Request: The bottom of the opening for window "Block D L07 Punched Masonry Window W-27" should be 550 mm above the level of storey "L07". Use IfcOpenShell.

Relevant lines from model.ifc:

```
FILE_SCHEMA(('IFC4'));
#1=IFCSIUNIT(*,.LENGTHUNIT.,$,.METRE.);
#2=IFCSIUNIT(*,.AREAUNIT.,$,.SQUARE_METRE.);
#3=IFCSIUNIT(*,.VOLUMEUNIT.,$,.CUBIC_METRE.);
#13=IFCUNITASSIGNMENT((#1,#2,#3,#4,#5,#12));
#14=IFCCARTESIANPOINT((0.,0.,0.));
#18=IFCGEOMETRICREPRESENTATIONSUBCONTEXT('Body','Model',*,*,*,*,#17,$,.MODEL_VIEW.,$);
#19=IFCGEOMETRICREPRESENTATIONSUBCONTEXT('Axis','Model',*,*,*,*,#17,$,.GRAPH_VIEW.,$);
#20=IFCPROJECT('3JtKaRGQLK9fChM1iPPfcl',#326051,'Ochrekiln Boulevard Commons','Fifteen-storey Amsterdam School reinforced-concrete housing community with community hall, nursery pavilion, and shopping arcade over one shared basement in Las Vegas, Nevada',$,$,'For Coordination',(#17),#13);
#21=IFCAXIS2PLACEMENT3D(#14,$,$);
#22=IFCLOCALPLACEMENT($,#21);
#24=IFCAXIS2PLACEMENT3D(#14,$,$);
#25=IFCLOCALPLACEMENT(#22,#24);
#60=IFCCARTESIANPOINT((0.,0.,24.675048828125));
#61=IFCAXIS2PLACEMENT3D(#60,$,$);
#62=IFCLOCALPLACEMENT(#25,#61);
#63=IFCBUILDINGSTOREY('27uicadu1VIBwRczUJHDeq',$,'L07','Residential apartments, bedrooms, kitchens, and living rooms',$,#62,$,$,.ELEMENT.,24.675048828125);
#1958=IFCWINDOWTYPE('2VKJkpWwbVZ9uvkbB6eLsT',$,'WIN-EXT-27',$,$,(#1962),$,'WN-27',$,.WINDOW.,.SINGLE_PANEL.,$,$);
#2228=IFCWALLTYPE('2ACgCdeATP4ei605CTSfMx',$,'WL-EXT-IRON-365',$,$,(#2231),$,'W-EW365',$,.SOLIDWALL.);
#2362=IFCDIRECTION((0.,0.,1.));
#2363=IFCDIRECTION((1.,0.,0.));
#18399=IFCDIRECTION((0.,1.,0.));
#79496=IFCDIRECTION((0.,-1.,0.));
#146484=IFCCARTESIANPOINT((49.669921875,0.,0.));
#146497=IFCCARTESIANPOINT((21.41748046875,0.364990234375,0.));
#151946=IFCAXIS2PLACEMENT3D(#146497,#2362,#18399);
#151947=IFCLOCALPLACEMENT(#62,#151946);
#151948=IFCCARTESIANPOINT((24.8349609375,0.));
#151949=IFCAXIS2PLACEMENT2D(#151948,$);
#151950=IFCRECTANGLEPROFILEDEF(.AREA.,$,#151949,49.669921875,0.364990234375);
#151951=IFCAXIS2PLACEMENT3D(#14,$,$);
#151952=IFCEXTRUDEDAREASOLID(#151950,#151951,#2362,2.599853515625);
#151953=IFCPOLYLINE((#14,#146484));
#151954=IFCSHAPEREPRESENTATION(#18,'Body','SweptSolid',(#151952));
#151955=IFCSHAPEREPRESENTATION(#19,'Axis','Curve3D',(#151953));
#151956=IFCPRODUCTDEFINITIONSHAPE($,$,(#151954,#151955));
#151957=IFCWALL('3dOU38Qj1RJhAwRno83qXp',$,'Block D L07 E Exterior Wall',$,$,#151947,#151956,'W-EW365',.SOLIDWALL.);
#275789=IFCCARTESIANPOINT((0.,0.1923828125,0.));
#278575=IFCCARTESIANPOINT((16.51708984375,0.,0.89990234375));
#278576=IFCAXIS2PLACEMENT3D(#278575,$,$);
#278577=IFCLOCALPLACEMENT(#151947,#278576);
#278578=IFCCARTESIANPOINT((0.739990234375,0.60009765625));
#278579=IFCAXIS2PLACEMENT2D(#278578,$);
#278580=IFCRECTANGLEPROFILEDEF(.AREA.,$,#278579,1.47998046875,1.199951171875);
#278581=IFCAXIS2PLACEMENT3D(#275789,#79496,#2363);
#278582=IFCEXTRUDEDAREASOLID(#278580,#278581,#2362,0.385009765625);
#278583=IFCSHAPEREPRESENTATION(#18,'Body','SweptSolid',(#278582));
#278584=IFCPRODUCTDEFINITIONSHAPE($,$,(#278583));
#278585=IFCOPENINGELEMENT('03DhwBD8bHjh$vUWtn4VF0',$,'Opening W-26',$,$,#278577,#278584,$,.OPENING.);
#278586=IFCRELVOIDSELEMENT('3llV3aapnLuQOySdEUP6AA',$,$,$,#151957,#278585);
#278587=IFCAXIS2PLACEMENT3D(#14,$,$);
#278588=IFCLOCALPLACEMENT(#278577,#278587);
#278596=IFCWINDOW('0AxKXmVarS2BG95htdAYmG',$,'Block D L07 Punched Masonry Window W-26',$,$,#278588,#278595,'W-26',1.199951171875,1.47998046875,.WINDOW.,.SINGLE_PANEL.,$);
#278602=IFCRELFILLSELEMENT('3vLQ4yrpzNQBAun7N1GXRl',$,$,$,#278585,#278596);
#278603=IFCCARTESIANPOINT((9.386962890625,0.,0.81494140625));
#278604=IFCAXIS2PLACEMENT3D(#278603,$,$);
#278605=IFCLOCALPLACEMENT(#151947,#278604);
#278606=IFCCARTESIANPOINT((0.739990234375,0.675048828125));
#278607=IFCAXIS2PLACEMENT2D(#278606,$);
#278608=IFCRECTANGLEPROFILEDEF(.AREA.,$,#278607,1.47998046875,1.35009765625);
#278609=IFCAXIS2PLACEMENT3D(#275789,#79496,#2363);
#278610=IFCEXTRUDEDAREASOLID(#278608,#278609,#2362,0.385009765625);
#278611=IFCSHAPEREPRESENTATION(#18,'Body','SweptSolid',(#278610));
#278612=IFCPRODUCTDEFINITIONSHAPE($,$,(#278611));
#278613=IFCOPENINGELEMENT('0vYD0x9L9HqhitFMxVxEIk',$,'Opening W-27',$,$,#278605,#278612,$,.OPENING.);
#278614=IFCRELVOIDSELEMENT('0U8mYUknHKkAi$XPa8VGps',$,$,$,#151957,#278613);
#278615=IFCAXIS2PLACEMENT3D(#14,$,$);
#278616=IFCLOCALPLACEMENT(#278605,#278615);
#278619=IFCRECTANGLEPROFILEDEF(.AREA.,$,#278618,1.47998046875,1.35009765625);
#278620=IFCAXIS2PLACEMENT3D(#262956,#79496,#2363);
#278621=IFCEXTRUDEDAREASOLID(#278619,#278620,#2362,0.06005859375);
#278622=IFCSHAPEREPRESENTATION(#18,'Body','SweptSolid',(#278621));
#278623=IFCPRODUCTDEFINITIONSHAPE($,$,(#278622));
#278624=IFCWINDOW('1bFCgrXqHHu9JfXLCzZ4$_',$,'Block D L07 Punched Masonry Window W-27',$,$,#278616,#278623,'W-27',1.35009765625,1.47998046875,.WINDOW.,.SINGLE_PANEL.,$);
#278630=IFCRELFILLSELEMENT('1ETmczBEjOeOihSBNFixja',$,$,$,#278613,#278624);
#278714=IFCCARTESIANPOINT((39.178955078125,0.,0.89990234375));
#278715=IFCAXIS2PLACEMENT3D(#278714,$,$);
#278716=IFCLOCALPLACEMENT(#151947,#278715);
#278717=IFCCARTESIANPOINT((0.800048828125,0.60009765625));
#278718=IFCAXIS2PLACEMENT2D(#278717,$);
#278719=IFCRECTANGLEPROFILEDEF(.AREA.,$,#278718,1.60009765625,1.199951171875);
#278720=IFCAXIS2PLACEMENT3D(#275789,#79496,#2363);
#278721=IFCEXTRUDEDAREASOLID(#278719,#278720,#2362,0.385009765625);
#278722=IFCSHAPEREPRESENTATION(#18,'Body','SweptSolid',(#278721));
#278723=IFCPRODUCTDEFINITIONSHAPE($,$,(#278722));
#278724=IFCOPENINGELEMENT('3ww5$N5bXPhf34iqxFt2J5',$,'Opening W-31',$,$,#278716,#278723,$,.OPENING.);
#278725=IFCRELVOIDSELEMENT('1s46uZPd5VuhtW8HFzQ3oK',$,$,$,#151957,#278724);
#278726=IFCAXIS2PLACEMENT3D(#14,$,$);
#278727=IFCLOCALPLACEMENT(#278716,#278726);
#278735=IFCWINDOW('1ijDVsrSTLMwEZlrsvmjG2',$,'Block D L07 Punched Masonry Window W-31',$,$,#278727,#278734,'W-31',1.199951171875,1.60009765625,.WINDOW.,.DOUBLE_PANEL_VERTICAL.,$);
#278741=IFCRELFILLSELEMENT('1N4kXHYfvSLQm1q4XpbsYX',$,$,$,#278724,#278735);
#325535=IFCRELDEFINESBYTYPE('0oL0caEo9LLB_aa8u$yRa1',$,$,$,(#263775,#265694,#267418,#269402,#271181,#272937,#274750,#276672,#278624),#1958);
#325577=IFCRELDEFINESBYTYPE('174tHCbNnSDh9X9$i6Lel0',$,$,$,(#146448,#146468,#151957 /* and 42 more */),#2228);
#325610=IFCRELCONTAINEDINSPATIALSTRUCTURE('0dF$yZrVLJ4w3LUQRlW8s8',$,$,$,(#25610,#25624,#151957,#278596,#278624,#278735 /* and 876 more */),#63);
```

```python
import numpy as np
import ifcopenshell
import ifcopenshell.api.geometry
import ifcopenshell.geom
import ifcopenshell.util.element
import ifcopenshell.util.placement
import ifcopenshell.util.shape
import ifcopenshell.util.unit

model = ifcopenshell.open("model.ifc")
unit_scale = ifcopenshell.util.unit.calculate_unit_scale(model)

window = model.by_id(278624)
opening = window.FillsVoids[0].RelatingOpeningElement
storey = ifcopenshell.util.element.get_container(window, ifc_class="IfcBuildingStorey")
level = ifcopenshell.util.placement.get_local_placement(storey.ObjectPlacement)[2, 3]

# The opening's origin need not be at the sill, so measure its lowest point.
shape = ifcopenshell.geom.create_shape(ifcopenshell.geom.settings(), opening)
bottom = ifcopenshell.util.shape.get_shape_bottom_elevation(shape, shape.geometry) / unit_scale
dz = level + 0.55 / unit_scale - bottom

shift = np.array([0.0, 0.0, dz])
# The window is placed relative to its opening, so it follows when the opening moves.
matrix = ifcopenshell.util.placement.get_local_placement(opening.ObjectPlacement)
matrix[:3, 3] += shift
ifcopenshell.api.geometry.edit_object_placement(
    model, product=opening, matrix=matrix, is_si=False, should_transform_children=True
)

print(f"moved by {dz * unit_scale:+.3f} m")

model.write("model_rev.ifc")
```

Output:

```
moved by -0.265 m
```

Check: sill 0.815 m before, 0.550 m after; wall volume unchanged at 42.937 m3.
